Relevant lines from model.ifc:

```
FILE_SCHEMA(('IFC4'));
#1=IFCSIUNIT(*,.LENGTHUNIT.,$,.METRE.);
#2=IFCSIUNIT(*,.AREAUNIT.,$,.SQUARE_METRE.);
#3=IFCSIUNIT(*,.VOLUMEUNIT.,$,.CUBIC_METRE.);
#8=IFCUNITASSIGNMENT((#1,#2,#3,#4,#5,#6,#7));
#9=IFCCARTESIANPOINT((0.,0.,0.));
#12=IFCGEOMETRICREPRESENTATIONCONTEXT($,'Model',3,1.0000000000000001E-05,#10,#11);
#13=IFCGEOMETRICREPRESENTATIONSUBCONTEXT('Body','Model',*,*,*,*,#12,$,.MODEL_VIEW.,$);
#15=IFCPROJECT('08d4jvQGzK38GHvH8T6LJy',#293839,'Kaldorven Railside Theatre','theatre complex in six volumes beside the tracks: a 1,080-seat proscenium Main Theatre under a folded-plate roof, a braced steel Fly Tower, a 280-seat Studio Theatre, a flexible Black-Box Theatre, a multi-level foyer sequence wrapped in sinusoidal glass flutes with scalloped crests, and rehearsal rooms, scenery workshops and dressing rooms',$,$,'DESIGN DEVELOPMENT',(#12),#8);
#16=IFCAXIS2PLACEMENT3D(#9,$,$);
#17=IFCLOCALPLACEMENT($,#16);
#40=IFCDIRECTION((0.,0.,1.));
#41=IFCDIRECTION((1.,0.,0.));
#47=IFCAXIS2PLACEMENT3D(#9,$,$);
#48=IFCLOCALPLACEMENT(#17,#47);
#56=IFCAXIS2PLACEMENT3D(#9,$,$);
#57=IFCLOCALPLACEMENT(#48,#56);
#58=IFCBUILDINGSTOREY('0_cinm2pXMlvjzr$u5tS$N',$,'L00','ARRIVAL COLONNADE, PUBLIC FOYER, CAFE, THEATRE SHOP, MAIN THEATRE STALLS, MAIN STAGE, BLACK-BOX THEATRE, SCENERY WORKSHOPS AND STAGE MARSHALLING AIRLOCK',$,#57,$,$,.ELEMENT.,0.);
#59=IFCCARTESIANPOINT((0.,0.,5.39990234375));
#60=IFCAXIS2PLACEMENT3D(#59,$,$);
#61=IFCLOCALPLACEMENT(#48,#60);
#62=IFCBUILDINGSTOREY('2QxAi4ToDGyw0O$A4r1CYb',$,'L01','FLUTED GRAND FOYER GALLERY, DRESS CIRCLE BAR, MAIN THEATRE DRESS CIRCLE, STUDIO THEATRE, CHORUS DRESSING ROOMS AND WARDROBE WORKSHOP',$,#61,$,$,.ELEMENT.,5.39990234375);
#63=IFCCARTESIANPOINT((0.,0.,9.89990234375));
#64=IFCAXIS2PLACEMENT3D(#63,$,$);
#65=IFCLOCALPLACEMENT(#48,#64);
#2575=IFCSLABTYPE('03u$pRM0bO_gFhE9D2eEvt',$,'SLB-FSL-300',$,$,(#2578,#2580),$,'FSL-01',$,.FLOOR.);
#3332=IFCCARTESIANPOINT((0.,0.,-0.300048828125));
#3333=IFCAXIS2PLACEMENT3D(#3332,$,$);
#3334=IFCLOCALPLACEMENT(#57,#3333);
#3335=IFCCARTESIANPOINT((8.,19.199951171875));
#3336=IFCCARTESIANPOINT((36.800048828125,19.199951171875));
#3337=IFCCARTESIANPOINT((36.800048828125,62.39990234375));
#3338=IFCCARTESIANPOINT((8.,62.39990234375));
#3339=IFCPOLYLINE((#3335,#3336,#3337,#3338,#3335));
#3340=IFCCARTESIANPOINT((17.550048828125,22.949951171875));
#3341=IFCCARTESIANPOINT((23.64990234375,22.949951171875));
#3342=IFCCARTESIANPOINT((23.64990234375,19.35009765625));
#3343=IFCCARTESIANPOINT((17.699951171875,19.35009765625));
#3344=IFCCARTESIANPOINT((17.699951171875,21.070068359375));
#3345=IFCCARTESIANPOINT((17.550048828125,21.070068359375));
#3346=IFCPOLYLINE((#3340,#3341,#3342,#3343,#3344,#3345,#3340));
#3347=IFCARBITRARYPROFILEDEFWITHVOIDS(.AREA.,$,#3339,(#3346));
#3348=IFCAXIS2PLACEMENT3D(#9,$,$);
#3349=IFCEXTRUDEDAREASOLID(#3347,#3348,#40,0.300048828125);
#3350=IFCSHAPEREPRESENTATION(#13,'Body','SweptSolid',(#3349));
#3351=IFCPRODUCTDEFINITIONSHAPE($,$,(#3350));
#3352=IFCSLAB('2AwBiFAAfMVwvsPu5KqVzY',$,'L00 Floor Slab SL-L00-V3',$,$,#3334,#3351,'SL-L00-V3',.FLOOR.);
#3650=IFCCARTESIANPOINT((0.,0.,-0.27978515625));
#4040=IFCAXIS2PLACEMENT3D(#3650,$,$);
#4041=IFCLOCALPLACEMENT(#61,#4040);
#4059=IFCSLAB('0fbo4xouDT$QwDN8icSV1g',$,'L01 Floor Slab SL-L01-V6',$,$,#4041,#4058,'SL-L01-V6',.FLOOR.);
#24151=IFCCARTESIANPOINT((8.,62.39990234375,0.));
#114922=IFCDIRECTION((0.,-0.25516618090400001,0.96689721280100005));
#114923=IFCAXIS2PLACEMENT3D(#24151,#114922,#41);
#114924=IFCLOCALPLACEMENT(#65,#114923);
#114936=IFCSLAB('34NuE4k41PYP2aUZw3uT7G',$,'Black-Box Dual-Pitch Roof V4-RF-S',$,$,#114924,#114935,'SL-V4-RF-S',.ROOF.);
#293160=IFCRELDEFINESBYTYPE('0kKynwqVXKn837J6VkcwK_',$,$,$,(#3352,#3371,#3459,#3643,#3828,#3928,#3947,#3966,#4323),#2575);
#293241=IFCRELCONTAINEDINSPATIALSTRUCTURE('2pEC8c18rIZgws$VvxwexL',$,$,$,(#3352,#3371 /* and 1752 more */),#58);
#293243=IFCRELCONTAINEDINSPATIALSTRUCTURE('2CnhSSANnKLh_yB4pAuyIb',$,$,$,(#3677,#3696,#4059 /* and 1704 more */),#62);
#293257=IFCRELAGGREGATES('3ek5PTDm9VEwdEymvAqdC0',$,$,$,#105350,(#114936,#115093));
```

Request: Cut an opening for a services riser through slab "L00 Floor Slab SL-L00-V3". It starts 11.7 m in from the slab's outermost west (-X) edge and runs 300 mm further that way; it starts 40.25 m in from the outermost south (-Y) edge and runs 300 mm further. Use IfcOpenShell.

```python
import numpy as np
import ifcopenshell
import ifcopenshell.api.feature
import ifcopenshell.api.geometry
import ifcopenshell.api.root
import ifcopenshell.geom
import ifcopenshell.util.placement
import ifcopenshell.util.representation
import ifcopenshell.util.shape
import ifcopenshell.util.unit

model = ifcopenshell.open("model.ifc")
unit_scale = ifcopenshell.util.unit.calculate_unit_scale(model)
settings = ifcopenshell.geom.settings()


def volume(element):
    """Net volume in cubic metres, openings subtracted."""
    shape = ifcopenshell.geom.create_shape(settings, element)
    return ifcopenshell.util.shape.get_volume(shape.geometry)


slab = model.by_guid("2AwBiFAAfMVwvsPu5KqVzY")
before = volume(slab)

# Extent in the slab's own axes, in metres. The edges named are its -X and -Y sides.
slab_shape = ifcopenshell.geom.create_shape(settings, slab)
vertices = ifcopenshell.util.shape.get_vertices(slab_shape.geometry)
x_min, y_min, bottom = vertices.min(axis=0)
top = vertices[:, 2].max()

opening = ifcopenshell.api.root.create_entity(model, ifc_class="IfcOpeningElement", name="Services riser opening", predefined_type="OPENING")
context = ifcopenshell.util.representation.get_context(model, "Model", "Body", "MODEL_VIEW")
width, depth = 0.3, 0.3
outline = [(0.0, 0.0), (width, 0.0), (width, depth), (0.0, depth), (0.0, 0.0)]
# Overshoot both faces by 50 mm so the cut is clean.
shape = ifcopenshell.api.geometry.add_slab_representation(
    model, context=context, depth=top - bottom + 0.1, polyline=outline
)
ifcopenshell.api.geometry.assign_representation(model, product=opening, representation=shape)

matrix = ifcopenshell.util.placement.get_local_placement(slab.ObjectPlacement)
matrix[:, 3] = matrix @ np.append(np.array([x_min + 11.7, y_min + 40.25, bottom - 0.05]) / unit_scale, 1.0)
ifcopenshell.api.geometry.edit_object_placement(model, product=opening, matrix=matrix, is_si=False)
ifcopenshell.api.feature.add_feature(model, feature=opening, element=slab)

after = volume(slab)

print(f"slab volume {before:.3f} -> {after:.3f} m3")

model.write("model_rev.ifc")
```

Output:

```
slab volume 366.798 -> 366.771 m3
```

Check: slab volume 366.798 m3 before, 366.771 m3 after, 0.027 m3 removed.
